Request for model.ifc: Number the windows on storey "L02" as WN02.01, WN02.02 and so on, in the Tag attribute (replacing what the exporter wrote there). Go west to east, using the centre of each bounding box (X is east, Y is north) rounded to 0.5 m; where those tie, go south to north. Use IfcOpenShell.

First a look at what the model holds.

```python
import ifcopenshell
import ifcopenshell.util.element
import ifcopenshell.util.placement

model = ifcopenshell.open("model.ifc")
print(model.schema)
storey = next(s for s in model.by_type("IfcBuildingStorey") if s.Name == "L02")
windows = [e for e in ifcopenshell.util.element.get_decomposition(storey) if e.is_a("IfcWindow")]
for e in sorted(windows, key=lambda e: e.id()):
    origin = ifcopenshell.util.placement.get_local_placement(e.ObjectPlacement)[:3, 3]
    print(e.id(), e.Tag, e.Name, origin.round(2) + 0.0, sep=" | ")
```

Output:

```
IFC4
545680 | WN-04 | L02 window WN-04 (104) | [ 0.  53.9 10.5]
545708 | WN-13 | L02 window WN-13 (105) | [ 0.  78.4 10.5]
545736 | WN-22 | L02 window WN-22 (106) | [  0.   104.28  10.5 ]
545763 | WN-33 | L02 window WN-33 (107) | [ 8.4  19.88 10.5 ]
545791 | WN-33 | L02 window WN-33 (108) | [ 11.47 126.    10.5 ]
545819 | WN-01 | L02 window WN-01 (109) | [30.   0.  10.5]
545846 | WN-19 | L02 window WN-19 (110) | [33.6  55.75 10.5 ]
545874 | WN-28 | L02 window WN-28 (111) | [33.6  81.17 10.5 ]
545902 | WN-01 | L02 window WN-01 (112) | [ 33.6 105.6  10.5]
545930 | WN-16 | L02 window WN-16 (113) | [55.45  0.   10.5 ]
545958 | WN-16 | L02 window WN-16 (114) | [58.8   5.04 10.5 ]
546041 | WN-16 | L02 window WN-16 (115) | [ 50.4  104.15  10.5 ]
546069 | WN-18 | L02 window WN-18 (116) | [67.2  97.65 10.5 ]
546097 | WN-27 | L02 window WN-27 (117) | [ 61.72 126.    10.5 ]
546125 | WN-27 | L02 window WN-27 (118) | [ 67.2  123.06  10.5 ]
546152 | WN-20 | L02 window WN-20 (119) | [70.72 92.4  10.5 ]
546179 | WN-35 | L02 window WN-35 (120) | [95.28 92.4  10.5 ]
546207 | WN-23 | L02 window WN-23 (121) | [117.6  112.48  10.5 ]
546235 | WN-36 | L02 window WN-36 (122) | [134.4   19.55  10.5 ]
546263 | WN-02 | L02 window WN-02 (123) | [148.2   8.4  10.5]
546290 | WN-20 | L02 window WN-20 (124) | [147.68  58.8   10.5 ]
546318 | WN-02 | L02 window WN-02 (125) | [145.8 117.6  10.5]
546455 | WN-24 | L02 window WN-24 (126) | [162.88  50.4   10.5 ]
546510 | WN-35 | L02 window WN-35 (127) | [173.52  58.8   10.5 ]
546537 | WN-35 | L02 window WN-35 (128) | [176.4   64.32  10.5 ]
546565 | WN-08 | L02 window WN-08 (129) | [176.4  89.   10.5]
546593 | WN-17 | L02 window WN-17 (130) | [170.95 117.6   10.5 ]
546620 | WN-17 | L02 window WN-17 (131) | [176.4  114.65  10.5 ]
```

```python
import ifcopenshell
import ifcopenshell.geom
import ifcopenshell.util.element
import ifcopenshell.util.shape

model = ifcopenshell.open("model.ifc")
settings = ifcopenshell.geom.settings()
settings.set("use-world-coords", True)


def centre(element):
    shape = ifcopenshell.geom.create_shape(settings, element)
    return ifcopenshell.util.shape.get_bbox_centroid(shape.geometry)


storey = next(s for s in model.by_type("IfcBuildingStorey") if s.Name == "L02")
windows = [e for e in ifcopenshell.util.element.get_decomposition(storey) if e.is_a("IfcWindow")]

# Insertion points can sit at a corner or the storey origin, so sort by the geometry (in metres).
centres = {e: centre(e) for e in windows}
windows.sort(key=lambda e: (round(centres[e][0] / 0.5), centres[e][1]))

for i, e in enumerate(windows, start=1):
    number = f"WN02.{i:02d}"
    e.Tag = number
    print(e.id(), number)

model.write("model-out.ifc")
```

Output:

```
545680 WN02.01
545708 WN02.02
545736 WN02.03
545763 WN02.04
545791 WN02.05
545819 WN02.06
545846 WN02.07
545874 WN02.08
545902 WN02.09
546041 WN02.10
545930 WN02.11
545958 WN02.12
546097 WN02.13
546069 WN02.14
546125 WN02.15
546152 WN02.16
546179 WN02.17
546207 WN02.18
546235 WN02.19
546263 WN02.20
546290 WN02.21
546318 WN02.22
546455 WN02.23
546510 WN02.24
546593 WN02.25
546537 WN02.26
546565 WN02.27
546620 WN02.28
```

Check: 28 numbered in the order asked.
